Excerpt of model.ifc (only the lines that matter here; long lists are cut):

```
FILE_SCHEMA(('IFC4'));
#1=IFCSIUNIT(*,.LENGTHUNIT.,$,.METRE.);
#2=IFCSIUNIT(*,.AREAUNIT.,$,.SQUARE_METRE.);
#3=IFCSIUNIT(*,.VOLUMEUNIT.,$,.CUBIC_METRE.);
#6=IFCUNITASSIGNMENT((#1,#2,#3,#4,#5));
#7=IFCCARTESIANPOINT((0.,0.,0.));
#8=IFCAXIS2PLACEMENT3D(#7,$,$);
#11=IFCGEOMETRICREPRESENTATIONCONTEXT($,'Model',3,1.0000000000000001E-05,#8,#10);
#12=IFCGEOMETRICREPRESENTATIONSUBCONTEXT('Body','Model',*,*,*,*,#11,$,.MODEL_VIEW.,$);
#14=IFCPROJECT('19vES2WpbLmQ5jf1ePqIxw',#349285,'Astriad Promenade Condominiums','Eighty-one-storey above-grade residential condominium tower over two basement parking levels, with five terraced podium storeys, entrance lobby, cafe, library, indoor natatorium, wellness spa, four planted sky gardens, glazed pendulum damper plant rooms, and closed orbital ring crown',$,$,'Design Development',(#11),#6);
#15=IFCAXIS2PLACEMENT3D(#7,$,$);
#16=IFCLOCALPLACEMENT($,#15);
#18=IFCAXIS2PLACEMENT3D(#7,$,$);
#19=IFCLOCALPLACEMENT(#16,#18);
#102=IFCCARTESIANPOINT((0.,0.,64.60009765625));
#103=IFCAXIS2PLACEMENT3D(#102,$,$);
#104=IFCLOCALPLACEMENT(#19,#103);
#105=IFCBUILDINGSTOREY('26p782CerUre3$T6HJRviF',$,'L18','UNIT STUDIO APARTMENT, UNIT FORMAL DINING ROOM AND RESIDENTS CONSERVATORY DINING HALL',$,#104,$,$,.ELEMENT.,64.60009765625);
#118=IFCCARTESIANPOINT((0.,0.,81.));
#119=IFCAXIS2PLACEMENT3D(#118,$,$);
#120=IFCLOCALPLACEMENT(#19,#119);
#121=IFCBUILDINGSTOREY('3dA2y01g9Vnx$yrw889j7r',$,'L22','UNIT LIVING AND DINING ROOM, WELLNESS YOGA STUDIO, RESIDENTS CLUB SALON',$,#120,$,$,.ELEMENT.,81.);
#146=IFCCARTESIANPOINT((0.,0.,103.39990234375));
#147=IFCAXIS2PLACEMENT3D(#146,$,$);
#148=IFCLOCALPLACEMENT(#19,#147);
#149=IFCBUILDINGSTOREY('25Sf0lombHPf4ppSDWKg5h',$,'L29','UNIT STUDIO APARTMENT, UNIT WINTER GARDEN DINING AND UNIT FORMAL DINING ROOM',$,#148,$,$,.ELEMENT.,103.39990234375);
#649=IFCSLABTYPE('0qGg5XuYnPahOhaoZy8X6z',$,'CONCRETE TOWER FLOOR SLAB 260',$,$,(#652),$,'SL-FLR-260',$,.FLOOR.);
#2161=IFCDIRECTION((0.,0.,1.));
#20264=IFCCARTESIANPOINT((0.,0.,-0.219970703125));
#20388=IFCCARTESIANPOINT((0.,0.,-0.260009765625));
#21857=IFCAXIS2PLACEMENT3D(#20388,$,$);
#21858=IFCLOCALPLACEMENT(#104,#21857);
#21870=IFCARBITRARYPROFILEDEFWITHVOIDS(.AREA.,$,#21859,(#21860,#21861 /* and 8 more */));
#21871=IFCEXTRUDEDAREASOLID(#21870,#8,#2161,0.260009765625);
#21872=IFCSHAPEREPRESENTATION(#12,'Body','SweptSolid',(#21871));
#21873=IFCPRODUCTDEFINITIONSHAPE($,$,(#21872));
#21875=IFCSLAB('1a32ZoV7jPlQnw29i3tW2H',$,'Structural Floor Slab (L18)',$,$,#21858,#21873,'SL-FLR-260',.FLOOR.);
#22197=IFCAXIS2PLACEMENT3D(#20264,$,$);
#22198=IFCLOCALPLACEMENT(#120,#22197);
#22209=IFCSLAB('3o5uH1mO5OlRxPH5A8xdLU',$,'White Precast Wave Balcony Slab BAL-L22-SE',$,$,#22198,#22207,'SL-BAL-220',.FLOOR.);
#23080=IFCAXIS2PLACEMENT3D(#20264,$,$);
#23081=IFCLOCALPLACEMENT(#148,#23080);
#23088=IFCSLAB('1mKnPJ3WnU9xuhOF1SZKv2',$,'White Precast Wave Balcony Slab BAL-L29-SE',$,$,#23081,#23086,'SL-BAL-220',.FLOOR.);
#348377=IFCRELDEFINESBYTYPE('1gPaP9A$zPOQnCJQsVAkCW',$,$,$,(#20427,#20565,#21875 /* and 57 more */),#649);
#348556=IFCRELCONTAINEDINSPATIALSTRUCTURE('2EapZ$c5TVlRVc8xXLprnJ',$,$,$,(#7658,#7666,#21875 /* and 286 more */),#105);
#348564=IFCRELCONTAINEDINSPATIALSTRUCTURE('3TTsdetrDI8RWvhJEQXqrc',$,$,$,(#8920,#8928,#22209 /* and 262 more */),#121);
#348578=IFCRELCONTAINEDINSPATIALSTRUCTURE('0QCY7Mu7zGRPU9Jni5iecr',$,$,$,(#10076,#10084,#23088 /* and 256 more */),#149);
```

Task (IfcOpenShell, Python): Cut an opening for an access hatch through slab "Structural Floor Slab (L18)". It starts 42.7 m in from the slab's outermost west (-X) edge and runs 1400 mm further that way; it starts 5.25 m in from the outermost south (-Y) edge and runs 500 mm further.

```python
import numpy as np
import ifcopenshell
import ifcopenshell.api.feature
import ifcopenshell.api.geometry
import ifcopenshell.api.root
import ifcopenshell.geom
import ifcopenshell.util.placement
import ifcopenshell.util.representation
import ifcopenshell.util.shape
import ifcopenshell.util.unit

model = ifcopenshell.open("model.ifc")
unit_scale = ifcopenshell.util.unit.calculate_unit_scale(model)
settings = ifcopenshell.geom.settings()


def volume(element):
    """Net volume in cubic metres, openings subtracted."""
    shape = ifcopenshell.geom.create_shape(settings, element)
    return ifcopenshell.util.shape.get_volume(shape.geometry)


slab = model.by_guid("1a32ZoV7jPlQnw29i3tW2H")
before = volume(slab)

# Extent in the slab's own axes, in metres. The edges named are its -X and -Y sides.
slab_shape = ifcopenshell.geom.create_shape(settings, slab)
vertices = ifcopenshell.util.shape.get_vertices(slab_shape.geometry)
x_min, y_min, bottom = vertices.min(axis=0)
top = vertices[:, 2].max()

opening = ifcopenshell.api.root.create_entity(model, ifc_class="IfcOpeningElement", name="Access hatch opening", predefined_type="OPENING")
context = ifcopenshell.util.representation.get_context(model, "Model", "Body", "MODEL_VIEW")
width, depth = 1.4, 0.5
outline = [(0.0, 0.0), (width, 0.0), (width, depth), (0.0, depth), (0.0, 0.0)]
# Overshoot both faces by 50 mm so the cut is clean.
shape = ifcopenshell.api.geometry.add_slab_representation(
    model, context=context, depth=top - bottom + 0.1, polyline=outline
)
ifcopenshell.api.geometry.assign_representation(model, product=opening, representation=shape)

matrix = ifcopenshell.util.placement.get_local_placement(slab.ObjectPlacement)
matrix[:, 3] = matrix @ np.append(np.array([x_min + 42.7, y_min + 5.25, bottom - 0.05]) / unit_scale, 1.0)
ifcopenshell.api.geometry.edit_object_placement(model, product=opening, matrix=matrix, is_si=False)
ifcopenshell.api.feature.add_feature(model, feature=opening, element=slab)

after = volume(slab)

print(f"slab volume {before:.3f} -> {after:.3f} m3")

model.write("model_edited.ifc")
```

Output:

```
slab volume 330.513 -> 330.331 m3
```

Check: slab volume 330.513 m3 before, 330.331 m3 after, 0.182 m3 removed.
